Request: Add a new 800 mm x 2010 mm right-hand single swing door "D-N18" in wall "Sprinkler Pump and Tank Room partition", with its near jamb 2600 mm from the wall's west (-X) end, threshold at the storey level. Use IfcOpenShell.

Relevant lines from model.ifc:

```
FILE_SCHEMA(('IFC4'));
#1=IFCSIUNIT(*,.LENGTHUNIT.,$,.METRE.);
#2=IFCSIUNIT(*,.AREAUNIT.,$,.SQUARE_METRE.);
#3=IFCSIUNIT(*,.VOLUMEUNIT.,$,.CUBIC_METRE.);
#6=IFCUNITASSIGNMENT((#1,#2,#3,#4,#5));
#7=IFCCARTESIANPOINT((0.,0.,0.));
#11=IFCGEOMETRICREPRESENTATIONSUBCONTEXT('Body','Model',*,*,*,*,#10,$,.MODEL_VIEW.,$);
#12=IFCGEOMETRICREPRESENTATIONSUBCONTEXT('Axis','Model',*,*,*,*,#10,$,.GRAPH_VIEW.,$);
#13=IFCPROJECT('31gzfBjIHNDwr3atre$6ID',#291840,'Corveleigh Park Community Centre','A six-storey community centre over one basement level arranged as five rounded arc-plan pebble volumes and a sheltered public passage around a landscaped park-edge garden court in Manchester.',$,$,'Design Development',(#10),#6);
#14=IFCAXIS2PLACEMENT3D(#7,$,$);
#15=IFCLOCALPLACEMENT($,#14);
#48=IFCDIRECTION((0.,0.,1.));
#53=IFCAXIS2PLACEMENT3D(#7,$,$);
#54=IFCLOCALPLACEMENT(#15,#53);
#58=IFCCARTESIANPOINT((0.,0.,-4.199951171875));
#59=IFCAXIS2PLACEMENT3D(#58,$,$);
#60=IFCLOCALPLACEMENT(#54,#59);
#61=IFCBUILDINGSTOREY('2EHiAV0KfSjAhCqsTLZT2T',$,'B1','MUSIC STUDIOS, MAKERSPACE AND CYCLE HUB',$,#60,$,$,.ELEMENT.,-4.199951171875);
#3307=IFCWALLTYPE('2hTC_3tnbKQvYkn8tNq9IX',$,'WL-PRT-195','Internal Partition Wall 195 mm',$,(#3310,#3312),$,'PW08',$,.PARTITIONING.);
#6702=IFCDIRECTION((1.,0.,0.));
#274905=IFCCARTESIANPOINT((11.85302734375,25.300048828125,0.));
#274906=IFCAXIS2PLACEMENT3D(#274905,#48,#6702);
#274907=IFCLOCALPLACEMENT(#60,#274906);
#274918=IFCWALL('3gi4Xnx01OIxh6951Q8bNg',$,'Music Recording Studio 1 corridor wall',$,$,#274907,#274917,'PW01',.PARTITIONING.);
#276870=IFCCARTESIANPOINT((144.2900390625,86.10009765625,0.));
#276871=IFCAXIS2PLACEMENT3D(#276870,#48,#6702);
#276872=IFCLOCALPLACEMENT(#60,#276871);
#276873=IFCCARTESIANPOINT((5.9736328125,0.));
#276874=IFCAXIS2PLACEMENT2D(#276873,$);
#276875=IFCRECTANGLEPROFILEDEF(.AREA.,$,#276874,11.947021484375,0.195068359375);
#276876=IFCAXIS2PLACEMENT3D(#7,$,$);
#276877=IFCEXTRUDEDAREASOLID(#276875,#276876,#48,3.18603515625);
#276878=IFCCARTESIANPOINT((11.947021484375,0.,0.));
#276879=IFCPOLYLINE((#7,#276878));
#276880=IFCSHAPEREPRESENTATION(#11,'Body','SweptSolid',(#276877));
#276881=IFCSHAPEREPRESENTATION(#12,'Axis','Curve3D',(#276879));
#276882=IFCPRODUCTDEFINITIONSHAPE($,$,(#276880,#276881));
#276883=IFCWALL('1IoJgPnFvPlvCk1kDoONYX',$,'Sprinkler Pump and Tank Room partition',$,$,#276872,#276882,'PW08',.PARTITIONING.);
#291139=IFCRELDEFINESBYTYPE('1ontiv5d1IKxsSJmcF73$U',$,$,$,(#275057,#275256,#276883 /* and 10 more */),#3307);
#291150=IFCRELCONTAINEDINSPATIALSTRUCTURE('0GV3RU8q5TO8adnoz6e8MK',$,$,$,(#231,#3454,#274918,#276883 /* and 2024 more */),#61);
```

```python
import numpy as np
import ifcopenshell
import ifcopenshell.api.feature
import ifcopenshell.api.geometry
import ifcopenshell.api.root
import ifcopenshell.api.spatial
import ifcopenshell.geom
import ifcopenshell.util.element
import ifcopenshell.util.placement
import ifcopenshell.util.representation
import ifcopenshell.util.shape
import ifcopenshell.util.unit

model = ifcopenshell.open("model.ifc")
unit_scale = ifcopenshell.util.unit.calculate_unit_scale(model)
settings = ifcopenshell.geom.settings()


def volume(element):
    """Net volume in cubic metres, openings subtracted."""
    shape = ifcopenshell.geom.create_shape(settings, element)
    return ifcopenshell.util.shape.get_volume(shape.geometry)


wall = model.by_guid("1IoJgPnFvPlvCk1kDoONYX")
storey = ifcopenshell.util.element.get_container(wall, ifc_class="IfcBuildingStorey")
context = ifcopenshell.util.representation.get_context(model, "Model", "Body", "MODEL_VIEW")
before = volume(wall)

width, height, from_end, sill = 0.8, 2.01, 2.6, 0.0  # metres

# The wall runs along its own X axis, and the end named is its -X end.
wall_shape = ifcopenshell.geom.create_shape(settings, wall)
x, y, z = ifcopenshell.util.shape.get_vertices(wall_shape.geometry).T
start = x.min() + from_end
face, thickness = float(y.min()), float(y.max() - y.min())
wall_matrix = ifcopenshell.util.placement.get_local_placement(wall.ObjectPlacement)
level = ifcopenshell.util.placement.get_local_placement(storey.ObjectPlacement)[2, 3]


def in_wall(x, y):
    """Placement at x, y metres in the wall's axes, at sill height."""
    matrix = wall_matrix.copy()
    matrix[:, 3] = wall_matrix @ np.array([x / unit_scale, y / unit_scale, 0.0, 1.0])
    matrix[2, 3] = level + sill / unit_scale
    return matrix


# Opening: a box that overshoots both wall faces by 50 mm.
opening = ifcopenshell.api.root.create_entity(model, ifc_class="IfcOpeningElement", predefined_type="OPENING")
box = ifcopenshell.api.geometry.add_wall_representation(
    model, context=context, length=width, height=height, thickness=thickness + 0.1
)
ifcopenshell.api.geometry.assign_representation(model, product=opening, representation=box)
ifcopenshell.api.geometry.edit_object_placement(model, product=opening, matrix=in_wall(start, face - 0.05), is_si=False)
ifcopenshell.api.feature.add_feature(model, feature=opening, element=wall)

door = ifcopenshell.api.root.create_entity(model, ifc_class="IfcDoor", name="D-N18", predefined_type="DOOR")
door.OverallWidth, door.OverallHeight = width / unit_scale, height / unit_scale
door.OperationType = "SINGLE_SWING_RIGHT"
body = ifcopenshell.api.geometry.add_door_representation(
    model,
    context=context,
    overall_width=door.OverallWidth,
    overall_height=door.OverallHeight,
    operation_type="SINGLE_SWING_RIGHT",
    lining_properties={"LiningDepth": thickness / unit_scale, "ThresholdDepth": thickness / unit_scale},
)
ifcopenshell.api.geometry.assign_representation(model, product=door, representation=body)
ifcopenshell.api.spatial.assign_container(model, products=[door], relating_structure=storey)
ifcopenshell.api.feature.add_filling(model, opening=opening, element=door)

# The lining spans the wall, so the door starts at the wall face.
ifcopenshell.api.geometry.edit_object_placement(model, product=door, matrix=in_wall(start, face), is_si=False)

after = volume(wall)

print(f"wall volume {before:.3f} -> {after:.3f} m3")

model.write("model-out.ifc")
```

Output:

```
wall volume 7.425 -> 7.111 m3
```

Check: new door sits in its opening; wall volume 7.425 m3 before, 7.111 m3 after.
